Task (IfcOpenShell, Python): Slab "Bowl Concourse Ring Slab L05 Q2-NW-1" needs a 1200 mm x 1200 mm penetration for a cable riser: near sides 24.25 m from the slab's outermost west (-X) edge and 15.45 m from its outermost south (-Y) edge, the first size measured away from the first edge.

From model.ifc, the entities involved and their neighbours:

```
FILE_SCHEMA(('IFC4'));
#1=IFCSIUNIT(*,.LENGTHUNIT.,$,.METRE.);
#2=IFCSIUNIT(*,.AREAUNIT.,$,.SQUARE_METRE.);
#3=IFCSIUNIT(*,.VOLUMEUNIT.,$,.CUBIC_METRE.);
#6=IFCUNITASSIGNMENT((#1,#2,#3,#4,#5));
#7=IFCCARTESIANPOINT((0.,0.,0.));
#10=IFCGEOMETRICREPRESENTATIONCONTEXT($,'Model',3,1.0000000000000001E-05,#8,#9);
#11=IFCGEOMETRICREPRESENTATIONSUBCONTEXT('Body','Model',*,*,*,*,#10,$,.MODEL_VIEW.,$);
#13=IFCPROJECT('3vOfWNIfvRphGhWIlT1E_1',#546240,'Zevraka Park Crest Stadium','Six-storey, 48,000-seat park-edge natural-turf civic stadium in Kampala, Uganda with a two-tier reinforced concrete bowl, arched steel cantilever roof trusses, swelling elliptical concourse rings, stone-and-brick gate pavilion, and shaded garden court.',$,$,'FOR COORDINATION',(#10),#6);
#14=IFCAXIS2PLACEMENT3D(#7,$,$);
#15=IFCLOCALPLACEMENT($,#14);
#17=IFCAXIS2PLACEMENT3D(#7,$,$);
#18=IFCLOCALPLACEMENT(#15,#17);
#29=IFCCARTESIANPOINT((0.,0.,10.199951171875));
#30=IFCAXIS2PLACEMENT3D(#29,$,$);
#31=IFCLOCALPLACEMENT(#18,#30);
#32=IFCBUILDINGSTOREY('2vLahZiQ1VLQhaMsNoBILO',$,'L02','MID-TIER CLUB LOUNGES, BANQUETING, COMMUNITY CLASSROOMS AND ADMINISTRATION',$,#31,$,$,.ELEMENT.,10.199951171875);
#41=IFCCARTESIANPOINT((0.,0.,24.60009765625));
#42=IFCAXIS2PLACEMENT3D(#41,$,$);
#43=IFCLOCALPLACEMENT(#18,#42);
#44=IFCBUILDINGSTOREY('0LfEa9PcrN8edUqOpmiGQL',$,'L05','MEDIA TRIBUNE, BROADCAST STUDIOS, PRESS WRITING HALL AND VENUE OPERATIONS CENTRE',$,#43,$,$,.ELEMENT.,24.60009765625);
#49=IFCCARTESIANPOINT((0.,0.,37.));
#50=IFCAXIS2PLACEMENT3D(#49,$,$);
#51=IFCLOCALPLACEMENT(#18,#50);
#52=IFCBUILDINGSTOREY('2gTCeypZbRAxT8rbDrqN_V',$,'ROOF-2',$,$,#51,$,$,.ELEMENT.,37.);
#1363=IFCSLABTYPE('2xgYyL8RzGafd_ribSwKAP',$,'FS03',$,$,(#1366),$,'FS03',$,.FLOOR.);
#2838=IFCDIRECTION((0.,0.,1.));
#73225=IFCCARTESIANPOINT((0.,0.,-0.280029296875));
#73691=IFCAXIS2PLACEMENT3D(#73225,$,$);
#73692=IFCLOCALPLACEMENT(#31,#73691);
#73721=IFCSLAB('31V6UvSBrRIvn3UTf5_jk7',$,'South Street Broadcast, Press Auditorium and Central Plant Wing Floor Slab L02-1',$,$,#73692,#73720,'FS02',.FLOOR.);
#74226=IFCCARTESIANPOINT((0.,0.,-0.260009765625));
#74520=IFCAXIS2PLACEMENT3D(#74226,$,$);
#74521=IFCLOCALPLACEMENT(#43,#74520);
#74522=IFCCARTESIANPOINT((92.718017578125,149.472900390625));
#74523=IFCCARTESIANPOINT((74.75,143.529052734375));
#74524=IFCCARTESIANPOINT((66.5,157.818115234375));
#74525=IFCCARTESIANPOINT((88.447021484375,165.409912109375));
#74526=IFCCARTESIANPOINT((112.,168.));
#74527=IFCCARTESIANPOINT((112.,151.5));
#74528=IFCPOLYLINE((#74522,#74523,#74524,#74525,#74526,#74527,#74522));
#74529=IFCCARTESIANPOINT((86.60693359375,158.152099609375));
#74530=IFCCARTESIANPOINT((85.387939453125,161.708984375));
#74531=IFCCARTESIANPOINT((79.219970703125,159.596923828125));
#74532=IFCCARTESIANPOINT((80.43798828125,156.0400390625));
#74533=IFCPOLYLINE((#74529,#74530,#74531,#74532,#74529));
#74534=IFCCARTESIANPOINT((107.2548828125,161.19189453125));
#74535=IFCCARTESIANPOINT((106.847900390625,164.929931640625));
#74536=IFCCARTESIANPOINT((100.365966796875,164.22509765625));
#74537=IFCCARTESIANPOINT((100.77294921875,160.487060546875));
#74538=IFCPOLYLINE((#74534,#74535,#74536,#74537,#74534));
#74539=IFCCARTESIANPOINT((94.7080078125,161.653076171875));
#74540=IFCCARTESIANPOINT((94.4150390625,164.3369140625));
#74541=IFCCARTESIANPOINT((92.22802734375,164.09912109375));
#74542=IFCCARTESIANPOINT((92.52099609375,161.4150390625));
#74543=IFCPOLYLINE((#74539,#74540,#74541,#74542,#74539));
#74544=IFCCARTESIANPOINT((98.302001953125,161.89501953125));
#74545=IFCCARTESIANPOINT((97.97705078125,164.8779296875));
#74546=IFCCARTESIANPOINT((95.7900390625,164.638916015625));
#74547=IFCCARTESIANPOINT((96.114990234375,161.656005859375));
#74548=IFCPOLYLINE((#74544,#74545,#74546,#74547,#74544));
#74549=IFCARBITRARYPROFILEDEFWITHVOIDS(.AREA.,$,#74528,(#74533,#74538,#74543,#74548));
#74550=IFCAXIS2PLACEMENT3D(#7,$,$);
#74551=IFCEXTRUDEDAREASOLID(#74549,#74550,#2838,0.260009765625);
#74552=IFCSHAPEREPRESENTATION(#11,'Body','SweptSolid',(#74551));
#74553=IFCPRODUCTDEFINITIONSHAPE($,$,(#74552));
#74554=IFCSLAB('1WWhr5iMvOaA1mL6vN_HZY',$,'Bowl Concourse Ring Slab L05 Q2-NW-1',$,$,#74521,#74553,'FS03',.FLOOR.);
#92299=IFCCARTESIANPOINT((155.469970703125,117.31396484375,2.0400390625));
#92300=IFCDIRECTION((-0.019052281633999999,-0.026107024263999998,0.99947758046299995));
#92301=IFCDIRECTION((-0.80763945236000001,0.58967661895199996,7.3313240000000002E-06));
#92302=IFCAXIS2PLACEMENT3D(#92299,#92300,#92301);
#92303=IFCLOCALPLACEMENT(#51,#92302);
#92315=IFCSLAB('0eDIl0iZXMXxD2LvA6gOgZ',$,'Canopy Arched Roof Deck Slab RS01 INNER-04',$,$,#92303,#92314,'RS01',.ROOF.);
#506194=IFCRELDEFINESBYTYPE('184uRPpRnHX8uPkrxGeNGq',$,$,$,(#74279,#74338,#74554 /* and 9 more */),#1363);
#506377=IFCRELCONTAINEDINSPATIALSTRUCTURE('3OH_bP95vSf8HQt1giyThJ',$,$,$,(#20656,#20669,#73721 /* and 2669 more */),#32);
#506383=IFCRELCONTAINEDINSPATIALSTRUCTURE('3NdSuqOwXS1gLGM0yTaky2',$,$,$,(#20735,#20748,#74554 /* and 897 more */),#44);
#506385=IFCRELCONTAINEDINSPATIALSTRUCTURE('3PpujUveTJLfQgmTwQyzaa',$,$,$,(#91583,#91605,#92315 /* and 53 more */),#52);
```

```python
import numpy as np
import ifcopenshell
import ifcopenshell.api.feature
import ifcopenshell.api.geometry
import ifcopenshell.api.root
import ifcopenshell.geom
import ifcopenshell.util.placement
import ifcopenshell.util.representation
import ifcopenshell.util.shape
import ifcopenshell.util.unit

model = ifcopenshell.open("model.ifc")
unit_scale = ifcopenshell.util.unit.calculate_unit_scale(model)
settings = ifcopenshell.geom.settings()


def volume(element):
    """Net volume in cubic metres, openings subtracted."""
    shape = ifcopenshell.geom.create_shape(settings, element)
    return ifcopenshell.util.shape.get_volume(shape.geometry)


slab = model.by_guid("1WWhr5iMvOaA1mL6vN_HZY")
before = volume(slab)

# Extent in the slab's own axes, in metres. The edges named are its -X and -Y sides.
slab_shape = ifcopenshell.geom.create_shape(settings, slab)
vertices = ifcopenshell.util.shape.get_vertices(slab_shape.geometry)
x_min, y_min, bottom = vertices.min(axis=0)
top = vertices[:, 2].max()

opening = ifcopenshell.api.root.create_entity(model, ifc_class="IfcOpeningElement", name="Cable riser opening", predefined_type="OPENING")
context = ifcopenshell.util.representation.get_context(model, "Model", "Body", "MODEL_VIEW")
width, depth = 1.2, 1.2
outline = [(0.0, 0.0), (width, 0.0), (width, depth), (0.0, depth), (0.0, 0.0)]
# Overshoot both faces by 50 mm so the cut is clean.
shape = ifcopenshell.api.geometry.add_slab_representation(
    model, context=context, depth=top - bottom + 0.1, polyline=outline
)
ifcopenshell.api.geometry.assign_representation(model, product=opening, representation=shape)

matrix = ifcopenshell.util.placement.get_local_placement(slab.ObjectPlacement)
matrix[:, 3] = matrix @ np.append(np.array([x_min + 24.25, y_min + 15.45, bottom - 0.05]) / unit_scale, 1.0)
ifcopenshell.api.geometry.edit_object_placement(model, product=opening, matrix=matrix, is_si=False)
ifcopenshell.api.feature.add_feature(model, feature=opening, element=slab)

after = volume(slab)

print(f"slab volume {before:.3f} -> {after:.3f} m3")

model.write("model_updated.ifc")
```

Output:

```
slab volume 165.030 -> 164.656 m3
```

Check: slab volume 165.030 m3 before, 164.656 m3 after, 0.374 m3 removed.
